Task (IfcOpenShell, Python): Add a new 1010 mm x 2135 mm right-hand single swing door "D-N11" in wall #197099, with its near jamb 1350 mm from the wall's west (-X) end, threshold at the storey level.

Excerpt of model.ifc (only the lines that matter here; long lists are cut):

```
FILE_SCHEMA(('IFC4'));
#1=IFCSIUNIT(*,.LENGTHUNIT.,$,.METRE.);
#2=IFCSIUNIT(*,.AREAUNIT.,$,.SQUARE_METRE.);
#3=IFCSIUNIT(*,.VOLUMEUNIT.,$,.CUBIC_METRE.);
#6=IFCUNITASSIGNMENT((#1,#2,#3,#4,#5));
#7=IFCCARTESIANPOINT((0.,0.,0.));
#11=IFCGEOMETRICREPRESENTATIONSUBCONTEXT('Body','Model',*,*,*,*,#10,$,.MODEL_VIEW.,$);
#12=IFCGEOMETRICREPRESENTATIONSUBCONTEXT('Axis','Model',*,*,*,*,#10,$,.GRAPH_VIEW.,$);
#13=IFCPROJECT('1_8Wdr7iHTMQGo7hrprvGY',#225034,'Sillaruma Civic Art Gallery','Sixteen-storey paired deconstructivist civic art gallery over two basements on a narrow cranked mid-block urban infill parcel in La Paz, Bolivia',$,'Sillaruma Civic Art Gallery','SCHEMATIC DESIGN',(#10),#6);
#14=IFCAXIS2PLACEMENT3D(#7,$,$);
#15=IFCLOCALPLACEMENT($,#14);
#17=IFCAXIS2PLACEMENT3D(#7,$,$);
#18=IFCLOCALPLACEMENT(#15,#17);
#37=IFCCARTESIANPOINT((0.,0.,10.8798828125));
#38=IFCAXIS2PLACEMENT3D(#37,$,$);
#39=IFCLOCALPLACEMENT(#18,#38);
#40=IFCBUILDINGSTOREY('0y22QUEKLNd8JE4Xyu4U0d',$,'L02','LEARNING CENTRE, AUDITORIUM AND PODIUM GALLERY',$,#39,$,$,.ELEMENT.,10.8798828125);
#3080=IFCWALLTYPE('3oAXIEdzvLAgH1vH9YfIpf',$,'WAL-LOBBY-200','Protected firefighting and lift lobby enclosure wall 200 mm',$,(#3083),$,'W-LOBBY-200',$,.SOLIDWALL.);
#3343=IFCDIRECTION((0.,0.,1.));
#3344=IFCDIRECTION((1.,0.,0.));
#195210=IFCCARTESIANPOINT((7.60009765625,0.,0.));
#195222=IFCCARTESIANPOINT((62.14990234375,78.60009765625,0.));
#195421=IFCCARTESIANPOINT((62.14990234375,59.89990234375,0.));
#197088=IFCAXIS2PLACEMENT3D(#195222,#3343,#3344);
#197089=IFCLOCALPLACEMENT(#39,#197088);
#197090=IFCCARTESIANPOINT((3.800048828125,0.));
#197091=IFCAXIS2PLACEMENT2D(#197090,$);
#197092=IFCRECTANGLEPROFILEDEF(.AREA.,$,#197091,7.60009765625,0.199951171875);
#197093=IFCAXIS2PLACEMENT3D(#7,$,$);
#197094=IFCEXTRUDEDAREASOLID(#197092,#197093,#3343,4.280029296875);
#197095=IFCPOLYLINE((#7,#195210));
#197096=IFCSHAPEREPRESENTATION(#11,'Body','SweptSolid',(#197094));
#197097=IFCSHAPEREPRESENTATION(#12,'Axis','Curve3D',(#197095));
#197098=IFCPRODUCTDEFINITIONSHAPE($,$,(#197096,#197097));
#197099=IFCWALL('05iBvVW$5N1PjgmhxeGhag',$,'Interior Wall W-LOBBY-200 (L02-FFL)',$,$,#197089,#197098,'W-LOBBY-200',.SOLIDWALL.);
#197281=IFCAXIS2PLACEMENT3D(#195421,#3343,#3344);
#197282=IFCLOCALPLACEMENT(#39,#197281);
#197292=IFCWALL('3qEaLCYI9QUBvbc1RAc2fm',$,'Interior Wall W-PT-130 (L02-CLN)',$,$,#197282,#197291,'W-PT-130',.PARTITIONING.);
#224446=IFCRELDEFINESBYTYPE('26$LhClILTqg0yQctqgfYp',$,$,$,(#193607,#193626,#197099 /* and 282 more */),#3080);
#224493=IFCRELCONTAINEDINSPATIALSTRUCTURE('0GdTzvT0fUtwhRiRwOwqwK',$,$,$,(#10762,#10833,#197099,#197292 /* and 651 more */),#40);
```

```python
import numpy as np
import ifcopenshell
import ifcopenshell.api.feature
import ifcopenshell.api.geometry
import ifcopenshell.api.root
import ifcopenshell.api.spatial
import ifcopenshell.geom
import ifcopenshell.util.element
import ifcopenshell.util.placement
import ifcopenshell.util.representation
import ifcopenshell.util.shape
import ifcopenshell.util.unit

model = ifcopenshell.open("model.ifc")
unit_scale = ifcopenshell.util.unit.calculate_unit_scale(model)
settings = ifcopenshell.geom.settings()


def volume(element):
    """Net volume in cubic metres, openings subtracted."""
    shape = ifcopenshell.geom.create_shape(settings, element)
    return ifcopenshell.util.shape.get_volume(shape.geometry)


wall = model.by_guid("05iBvVW$5N1PjgmhxeGhag")
storey = ifcopenshell.util.element.get_container(wall, ifc_class="IfcBuildingStorey")
context = ifcopenshell.util.representation.get_context(model, "Model", "Body", "MODEL_VIEW")
before = volume(wall)

width, height, from_end, sill = 1.01, 2.135, 1.35, 0.0  # metres

# The wall runs along its own X axis, and the end named is its -X end.
wall_shape = ifcopenshell.geom.create_shape(settings, wall)
x, y, z = ifcopenshell.util.shape.get_vertices(wall_shape.geometry).T
start = x.min() + from_end
face, thickness = float(y.min()), float(y.max() - y.min())
wall_matrix = ifcopenshell.util.placement.get_local_placement(wall.ObjectPlacement)
level = ifcopenshell.util.placement.get_local_placement(storey.ObjectPlacement)[2, 3]


def in_wall(x, y):
    """Placement at x, y metres in the wall's axes, at sill height."""
    matrix = wall_matrix.copy()
    matrix[:, 3] = wall_matrix @ np.array([x / unit_scale, y / unit_scale, 0.0, 1.0])
    matrix[2, 3] = level + sill / unit_scale
    return matrix


# Opening: a box that overshoots both wall faces by 50 mm.
opening = ifcopenshell.api.root.create_entity(model, ifc_class="IfcOpeningElement", predefined_type="OPENING")
box = ifcopenshell.api.geometry.add_wall_representation(
    model, context=context, length=width, height=height, thickness=thickness + 0.1
)
ifcopenshell.api.geometry.assign_representation(model, product=opening, representation=box)
ifcopenshell.api.geometry.edit_object_placement(model, product=opening, matrix=in_wall(start, face - 0.05), is_si=False)
ifcopenshell.api.feature.add_feature(model, feature=opening, element=wall)

door = ifcopenshell.api.root.create_entity(model, ifc_class="IfcDoor", name="D-N11", predefined_type="DOOR")
door.OverallWidth, door.OverallHeight = width / unit_scale, height / unit_scale
door.OperationType = "SINGLE_SWING_RIGHT"
body = ifcopenshell.api.geometry.add_door_representation(
    model,
    context=context,
    overall_width=door.OverallWidth,
    overall_height=door.OverallHeight,
    operation_type="SINGLE_SWING_RIGHT",
    lining_properties={"LiningDepth": thickness / unit_scale, "ThresholdDepth": thickness / unit_scale},
)
ifcopenshell.api.geometry.assign_representation(model, product=door, representation=body)
ifcopenshell.api.spatial.assign_container(model, products=[door], relating_structure=storey)
ifcopenshell.api.feature.add_filling(model, opening=opening, element=door)

# The lining spans the wall, so the door starts at the wall face.
ifcopenshell.api.geometry.edit_object_placement(model, product=door, matrix=in_wall(start, face), is_si=False)

after = volume(wall)

print(f"wall volume {before:.3f} -> {after:.3f} m3")

model.write("model-out.ifc")
```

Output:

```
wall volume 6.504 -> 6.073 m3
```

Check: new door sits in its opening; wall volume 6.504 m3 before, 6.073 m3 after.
